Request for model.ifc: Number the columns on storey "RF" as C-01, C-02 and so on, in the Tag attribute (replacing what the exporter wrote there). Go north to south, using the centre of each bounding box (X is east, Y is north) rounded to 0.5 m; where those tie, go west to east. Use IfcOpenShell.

First a look at what the model holds.

```python
import ifcopenshell
import ifcopenshell.util.element
import ifcopenshell.util.placement

model = ifcopenshell.open("model.ifc")
print(model.schema)
storey = next(s for s in model.by_type("IfcBuildingStorey") if s.Name == "RF")
columns = [e for e in ifcopenshell.util.element.get_decomposition(storey) if e.is_a("IfcColumn")]
for e in sorted(columns, key=lambda e: e.id()):
    origin = ifcopenshell.util.placement.get_local_placement(e.ObjectPlacement)[:3, 3]
    print(e.id(), e.Tag, e.Name, origin.round(2) + 0.0, sep=" | ")
```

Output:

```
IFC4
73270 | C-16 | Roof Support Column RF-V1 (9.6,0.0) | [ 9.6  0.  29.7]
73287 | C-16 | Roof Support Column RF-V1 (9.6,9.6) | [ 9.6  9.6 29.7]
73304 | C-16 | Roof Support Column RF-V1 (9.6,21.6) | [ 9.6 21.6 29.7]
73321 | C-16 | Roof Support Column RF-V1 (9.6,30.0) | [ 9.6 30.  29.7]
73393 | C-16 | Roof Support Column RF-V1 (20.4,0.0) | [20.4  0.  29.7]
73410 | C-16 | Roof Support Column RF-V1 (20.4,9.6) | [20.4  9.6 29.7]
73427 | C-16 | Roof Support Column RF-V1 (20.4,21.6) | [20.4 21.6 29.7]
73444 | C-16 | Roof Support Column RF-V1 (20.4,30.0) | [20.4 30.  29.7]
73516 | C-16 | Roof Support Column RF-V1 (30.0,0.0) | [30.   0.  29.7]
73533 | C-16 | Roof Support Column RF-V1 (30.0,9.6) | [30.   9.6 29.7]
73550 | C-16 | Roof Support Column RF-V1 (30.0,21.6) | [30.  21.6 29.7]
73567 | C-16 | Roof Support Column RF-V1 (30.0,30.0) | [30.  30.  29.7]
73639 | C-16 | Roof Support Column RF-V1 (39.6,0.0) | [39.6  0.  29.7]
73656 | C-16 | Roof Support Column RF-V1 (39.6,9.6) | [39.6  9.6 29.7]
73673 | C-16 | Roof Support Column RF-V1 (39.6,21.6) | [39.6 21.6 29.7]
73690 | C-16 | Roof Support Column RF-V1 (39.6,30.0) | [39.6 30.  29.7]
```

```python
import ifcopenshell
import ifcopenshell.geom
import ifcopenshell.util.element
import ifcopenshell.util.shape

model = ifcopenshell.open("model.ifc")
settings = ifcopenshell.geom.settings()
settings.set("use-world-coords", True)


def centre(element):
    shape = ifcopenshell.geom.create_shape(settings, element)
    return ifcopenshell.util.shape.get_bbox_centroid(shape.geometry)


storey = next(s for s in model.by_type("IfcBuildingStorey") if s.Name == "RF")
columns = [e for e in ifcopenshell.util.element.get_decomposition(storey) if e.is_a("IfcColumn")]

# Insertion points can sit at a corner or the storey origin, so sort by the geometry (in metres).
centres = {e: centre(e) for e in columns}
columns.sort(key=lambda e: (-round(centres[e][1] / 0.5), centres[e][0]))

for i, e in enumerate(columns, start=1):
    number = f"C-{i:02d}"
    e.Tag = number
    print(e.id(), number)

model.write("model-out.ifc")
```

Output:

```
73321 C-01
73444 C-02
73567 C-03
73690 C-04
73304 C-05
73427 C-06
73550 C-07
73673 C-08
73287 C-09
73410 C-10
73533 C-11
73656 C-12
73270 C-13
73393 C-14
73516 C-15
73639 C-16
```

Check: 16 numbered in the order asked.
